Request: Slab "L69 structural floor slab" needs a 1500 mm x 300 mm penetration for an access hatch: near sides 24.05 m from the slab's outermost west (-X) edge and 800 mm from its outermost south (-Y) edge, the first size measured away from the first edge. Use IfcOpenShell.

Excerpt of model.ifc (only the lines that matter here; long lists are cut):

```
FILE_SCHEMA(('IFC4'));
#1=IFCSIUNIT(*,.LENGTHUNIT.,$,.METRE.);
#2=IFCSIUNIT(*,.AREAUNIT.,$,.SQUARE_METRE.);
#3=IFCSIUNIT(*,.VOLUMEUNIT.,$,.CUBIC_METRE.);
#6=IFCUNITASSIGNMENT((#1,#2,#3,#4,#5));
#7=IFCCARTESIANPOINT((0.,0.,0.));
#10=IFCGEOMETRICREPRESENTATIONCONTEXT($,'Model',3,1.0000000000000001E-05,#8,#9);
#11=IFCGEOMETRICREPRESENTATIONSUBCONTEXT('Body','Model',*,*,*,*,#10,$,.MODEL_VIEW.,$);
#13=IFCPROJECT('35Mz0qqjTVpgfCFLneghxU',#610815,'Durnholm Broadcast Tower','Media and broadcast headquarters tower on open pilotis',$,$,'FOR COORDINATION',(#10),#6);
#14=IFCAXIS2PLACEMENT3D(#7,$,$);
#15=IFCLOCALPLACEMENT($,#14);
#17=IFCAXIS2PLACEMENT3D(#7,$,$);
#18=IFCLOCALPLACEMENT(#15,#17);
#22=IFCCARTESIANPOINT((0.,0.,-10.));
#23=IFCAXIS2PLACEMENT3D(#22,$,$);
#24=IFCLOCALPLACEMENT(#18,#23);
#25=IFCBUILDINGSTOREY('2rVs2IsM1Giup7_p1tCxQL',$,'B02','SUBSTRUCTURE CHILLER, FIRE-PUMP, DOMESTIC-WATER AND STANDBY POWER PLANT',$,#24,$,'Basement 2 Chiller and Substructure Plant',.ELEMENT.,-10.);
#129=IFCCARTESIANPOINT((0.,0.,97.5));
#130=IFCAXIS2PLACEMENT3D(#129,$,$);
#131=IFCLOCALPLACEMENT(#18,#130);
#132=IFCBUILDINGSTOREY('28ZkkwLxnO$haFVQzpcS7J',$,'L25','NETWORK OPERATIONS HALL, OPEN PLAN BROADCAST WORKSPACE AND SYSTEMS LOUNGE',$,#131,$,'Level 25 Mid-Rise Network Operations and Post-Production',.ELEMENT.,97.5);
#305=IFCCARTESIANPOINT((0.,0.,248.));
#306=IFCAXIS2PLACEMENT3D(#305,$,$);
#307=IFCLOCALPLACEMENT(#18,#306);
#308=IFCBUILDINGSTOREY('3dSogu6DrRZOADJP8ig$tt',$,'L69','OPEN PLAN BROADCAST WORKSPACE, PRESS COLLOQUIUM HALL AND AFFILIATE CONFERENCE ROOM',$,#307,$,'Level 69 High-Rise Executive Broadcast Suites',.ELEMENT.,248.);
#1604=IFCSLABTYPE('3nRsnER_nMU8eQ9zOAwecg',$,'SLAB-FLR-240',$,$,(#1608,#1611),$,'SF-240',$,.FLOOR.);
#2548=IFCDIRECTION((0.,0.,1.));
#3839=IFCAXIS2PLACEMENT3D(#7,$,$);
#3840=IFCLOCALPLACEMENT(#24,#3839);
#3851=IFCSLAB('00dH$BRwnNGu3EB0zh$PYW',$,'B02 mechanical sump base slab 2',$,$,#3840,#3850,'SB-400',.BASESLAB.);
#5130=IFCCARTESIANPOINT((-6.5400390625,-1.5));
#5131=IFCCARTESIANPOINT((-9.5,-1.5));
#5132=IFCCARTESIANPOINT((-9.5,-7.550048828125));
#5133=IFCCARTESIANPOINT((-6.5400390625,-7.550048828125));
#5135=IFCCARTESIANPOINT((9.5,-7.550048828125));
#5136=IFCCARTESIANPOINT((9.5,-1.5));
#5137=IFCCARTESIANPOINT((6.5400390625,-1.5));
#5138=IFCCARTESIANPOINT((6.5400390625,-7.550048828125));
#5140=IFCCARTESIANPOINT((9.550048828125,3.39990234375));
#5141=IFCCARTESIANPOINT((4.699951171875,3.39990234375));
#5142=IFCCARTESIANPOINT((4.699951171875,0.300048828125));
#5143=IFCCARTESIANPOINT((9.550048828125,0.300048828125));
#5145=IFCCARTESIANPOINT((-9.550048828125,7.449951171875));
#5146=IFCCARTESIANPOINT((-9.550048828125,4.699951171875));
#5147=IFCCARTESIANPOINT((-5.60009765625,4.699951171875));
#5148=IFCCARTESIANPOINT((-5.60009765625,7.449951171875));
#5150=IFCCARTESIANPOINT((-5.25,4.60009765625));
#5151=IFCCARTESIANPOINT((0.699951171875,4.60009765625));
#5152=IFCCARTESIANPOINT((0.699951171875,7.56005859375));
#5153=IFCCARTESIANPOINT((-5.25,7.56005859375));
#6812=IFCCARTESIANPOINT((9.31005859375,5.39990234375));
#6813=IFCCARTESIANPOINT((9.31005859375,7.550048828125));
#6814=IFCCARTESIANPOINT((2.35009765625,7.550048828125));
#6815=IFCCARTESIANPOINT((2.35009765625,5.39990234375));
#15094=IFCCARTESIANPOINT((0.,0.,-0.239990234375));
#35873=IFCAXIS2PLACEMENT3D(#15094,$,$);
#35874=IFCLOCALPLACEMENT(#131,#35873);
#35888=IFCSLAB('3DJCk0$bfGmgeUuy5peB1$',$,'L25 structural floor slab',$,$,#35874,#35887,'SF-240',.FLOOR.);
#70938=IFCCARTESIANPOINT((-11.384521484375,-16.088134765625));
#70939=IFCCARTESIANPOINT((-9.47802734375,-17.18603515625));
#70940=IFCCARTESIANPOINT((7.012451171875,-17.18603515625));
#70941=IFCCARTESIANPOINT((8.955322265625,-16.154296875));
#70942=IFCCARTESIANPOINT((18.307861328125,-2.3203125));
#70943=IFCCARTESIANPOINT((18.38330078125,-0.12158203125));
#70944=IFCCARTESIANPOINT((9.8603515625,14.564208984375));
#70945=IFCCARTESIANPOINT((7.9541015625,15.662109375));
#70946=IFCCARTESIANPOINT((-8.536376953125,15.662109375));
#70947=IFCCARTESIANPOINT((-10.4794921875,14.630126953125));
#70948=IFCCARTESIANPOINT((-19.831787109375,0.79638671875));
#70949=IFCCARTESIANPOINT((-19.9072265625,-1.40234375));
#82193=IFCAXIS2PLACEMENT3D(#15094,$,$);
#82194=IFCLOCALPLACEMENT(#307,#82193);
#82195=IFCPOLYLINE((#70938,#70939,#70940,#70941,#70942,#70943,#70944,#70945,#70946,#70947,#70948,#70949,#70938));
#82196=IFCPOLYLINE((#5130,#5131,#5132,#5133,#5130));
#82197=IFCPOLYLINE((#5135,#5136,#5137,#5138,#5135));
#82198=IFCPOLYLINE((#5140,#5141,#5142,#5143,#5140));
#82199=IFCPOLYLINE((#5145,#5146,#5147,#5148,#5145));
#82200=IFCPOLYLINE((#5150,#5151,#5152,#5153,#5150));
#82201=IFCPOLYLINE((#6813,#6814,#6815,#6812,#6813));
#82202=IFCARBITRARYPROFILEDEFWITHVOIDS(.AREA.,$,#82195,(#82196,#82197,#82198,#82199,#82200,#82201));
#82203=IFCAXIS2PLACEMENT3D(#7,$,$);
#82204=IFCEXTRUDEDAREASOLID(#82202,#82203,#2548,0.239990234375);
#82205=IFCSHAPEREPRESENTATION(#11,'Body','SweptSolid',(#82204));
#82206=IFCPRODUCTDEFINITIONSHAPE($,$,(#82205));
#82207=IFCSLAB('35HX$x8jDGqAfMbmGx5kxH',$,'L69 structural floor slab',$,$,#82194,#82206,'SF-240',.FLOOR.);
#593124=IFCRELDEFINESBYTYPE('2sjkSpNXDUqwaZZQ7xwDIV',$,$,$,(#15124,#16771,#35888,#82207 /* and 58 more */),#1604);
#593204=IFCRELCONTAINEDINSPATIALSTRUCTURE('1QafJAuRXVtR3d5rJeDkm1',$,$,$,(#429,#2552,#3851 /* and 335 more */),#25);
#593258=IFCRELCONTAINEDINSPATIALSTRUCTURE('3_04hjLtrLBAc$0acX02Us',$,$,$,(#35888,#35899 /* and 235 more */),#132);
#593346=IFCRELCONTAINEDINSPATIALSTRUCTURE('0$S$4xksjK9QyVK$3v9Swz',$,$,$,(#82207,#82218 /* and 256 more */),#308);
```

```python
import numpy as np
import ifcopenshell
import ifcopenshell.api.feature
import ifcopenshell.api.geometry
import ifcopenshell.api.root
import ifcopenshell.geom
import ifcopenshell.util.placement
import ifcopenshell.util.representation
import ifcopenshell.util.shape
import ifcopenshell.util.unit

model = ifcopenshell.open("model.ifc")
unit_scale = ifcopenshell.util.unit.calculate_unit_scale(model)
settings = ifcopenshell.geom.settings()


def volume(element):
    """Net volume in cubic metres, openings subtracted."""
    shape = ifcopenshell.geom.create_shape(settings, element)
    return ifcopenshell.util.shape.get_volume(shape.geometry)


slab = model.by_guid("35HX$x8jDGqAfMbmGx5kxH")
before = volume(slab)

# Extent in the slab's own axes, in metres. The edges named are its -X and -Y sides.
slab_shape = ifcopenshell.geom.create_shape(settings, slab)
vertices = ifcopenshell.util.shape.get_vertices(slab_shape.geometry)
x_min, y_min, bottom = vertices.min(axis=0)
top = vertices[:, 2].max()

opening = ifcopenshell.api.root.create_entity(model, ifc_class="IfcOpeningElement", name="Access hatch opening", predefined_type="OPENING")
context = ifcopenshell.util.representation.get_context(model, "Model", "Body", "MODEL_VIEW")
width, depth = 1.5, 0.3
outline = [(0.0, 0.0), (width, 0.0), (width, depth), (0.0, depth), (0.0, 0.0)]
# Overshoot both faces by 50 mm so the cut is clean.
shape = ifcopenshell.api.geometry.add_slab_representation(
    model, context=context, depth=top - bottom + 0.1, polyline=outline
)
ifcopenshell.api.geometry.assign_representation(model, product=opening, representation=shape)

matrix = ifcopenshell.util.placement.get_local_placement(slab.ObjectPlacement)
matrix[:, 3] = matrix @ np.append(np.array([x_min + 24.05, y_min + 0.8, bottom - 0.05]) / unit_scale, 1.0)
ifcopenshell.api.geometry.edit_object_placement(model, product=opening, matrix=matrix, is_si=False)
ifcopenshell.api.feature.add_feature(model, feature=opening, element=slab)

after = volume(slab)

print(f"slab volume {before:.3f} -> {after:.3f} m3")

model.write("model_edited.ifc")
```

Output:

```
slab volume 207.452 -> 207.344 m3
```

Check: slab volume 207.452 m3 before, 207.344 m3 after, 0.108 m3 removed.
